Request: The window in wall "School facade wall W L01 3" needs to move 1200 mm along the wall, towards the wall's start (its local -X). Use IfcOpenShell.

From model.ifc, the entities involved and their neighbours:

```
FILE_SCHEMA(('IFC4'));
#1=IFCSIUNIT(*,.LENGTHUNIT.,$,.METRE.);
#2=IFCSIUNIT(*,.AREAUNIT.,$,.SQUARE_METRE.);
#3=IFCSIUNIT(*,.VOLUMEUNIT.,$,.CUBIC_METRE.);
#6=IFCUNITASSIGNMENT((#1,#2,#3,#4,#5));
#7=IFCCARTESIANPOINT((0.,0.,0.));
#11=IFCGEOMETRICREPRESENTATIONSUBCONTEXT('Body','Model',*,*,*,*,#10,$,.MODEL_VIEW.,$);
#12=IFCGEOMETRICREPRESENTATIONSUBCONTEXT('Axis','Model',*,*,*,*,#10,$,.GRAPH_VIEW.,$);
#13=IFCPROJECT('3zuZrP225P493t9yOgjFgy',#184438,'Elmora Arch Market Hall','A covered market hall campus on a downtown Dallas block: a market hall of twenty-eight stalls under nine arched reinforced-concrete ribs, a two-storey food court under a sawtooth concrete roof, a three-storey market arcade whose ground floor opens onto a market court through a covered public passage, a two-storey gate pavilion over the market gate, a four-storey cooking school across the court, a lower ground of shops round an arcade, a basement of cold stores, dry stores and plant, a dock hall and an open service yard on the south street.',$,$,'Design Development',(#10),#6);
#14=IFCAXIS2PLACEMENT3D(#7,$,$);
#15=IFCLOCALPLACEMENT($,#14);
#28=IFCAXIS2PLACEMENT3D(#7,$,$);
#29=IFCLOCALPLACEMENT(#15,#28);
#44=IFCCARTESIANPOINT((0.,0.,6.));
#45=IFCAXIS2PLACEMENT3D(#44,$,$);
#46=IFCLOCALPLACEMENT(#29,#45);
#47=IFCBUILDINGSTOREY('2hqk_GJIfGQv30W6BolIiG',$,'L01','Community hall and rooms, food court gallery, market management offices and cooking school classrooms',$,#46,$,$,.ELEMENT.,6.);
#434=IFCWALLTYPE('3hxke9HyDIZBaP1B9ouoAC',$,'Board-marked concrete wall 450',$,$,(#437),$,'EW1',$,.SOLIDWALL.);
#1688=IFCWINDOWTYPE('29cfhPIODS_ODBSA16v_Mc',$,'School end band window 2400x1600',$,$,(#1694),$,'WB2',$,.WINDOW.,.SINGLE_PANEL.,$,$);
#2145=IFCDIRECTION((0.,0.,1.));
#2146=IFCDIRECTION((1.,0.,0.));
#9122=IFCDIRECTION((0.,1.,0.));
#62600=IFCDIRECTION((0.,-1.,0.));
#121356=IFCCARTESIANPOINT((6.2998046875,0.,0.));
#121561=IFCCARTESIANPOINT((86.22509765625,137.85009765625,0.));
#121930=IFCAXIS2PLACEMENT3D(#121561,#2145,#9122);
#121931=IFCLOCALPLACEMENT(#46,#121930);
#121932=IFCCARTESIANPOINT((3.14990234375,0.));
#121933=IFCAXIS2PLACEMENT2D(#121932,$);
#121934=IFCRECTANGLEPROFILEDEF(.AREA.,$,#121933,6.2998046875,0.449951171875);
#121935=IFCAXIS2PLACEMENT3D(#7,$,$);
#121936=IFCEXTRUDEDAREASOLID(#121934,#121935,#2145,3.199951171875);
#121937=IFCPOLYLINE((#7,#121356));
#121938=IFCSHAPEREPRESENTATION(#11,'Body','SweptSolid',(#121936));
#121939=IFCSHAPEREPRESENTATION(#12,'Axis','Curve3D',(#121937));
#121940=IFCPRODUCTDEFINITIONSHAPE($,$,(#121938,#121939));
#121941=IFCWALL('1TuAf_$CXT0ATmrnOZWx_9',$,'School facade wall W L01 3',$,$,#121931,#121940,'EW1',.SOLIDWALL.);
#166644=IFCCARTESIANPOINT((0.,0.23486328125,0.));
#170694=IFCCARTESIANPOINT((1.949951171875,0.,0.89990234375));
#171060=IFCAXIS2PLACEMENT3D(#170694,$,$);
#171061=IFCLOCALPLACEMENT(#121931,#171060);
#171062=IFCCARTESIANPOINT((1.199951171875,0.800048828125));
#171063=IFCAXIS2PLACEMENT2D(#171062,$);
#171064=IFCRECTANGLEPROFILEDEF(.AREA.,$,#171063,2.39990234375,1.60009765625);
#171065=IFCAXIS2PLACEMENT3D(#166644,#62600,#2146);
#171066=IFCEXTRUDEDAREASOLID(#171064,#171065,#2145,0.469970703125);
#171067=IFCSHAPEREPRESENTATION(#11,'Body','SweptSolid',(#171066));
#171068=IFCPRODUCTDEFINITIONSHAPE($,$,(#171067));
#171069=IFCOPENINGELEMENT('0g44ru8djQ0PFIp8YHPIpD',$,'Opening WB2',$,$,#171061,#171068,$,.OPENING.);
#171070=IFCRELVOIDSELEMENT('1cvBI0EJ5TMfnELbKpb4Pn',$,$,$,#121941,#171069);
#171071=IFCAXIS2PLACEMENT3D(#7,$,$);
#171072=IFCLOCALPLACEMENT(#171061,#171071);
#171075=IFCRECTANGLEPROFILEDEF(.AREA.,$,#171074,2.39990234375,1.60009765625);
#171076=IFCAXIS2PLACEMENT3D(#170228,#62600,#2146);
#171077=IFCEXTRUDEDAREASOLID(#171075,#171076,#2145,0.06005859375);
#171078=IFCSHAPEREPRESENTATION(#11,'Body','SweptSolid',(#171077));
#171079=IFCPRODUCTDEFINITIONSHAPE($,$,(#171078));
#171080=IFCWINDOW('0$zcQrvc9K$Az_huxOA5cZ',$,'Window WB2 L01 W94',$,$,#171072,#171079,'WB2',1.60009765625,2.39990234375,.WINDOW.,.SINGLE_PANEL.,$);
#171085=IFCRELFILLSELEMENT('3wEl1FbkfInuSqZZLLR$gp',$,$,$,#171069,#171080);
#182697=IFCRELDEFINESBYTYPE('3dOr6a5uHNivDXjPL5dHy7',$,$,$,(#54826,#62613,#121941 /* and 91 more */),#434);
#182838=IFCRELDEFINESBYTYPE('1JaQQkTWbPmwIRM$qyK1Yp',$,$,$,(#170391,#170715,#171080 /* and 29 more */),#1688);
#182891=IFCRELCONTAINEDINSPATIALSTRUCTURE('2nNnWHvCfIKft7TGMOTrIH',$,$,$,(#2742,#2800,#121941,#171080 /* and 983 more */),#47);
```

```python
import ifcopenshell
import ifcopenshell.api.geometry
import ifcopenshell.util.placement

model = ifcopenshell.open("model.ifc")

window = model.by_guid("0$zcQrvc9K$Az_huxOA5cZ")
opening = window.FillsVoids[0].RelatingOpeningElement
wall = opening.VoidsElements[0].RelatingBuildingElement

wall_matrix = ifcopenshell.util.placement.get_local_placement(wall.ObjectPlacement)
shift = wall_matrix[:3, 0] * -1.2
before = ifcopenshell.util.placement.get_local_placement(window.ObjectPlacement)[:3, 3].copy()

# The window is placed relative to its opening, so it follows when the opening moves.
matrix = ifcopenshell.util.placement.get_local_placement(opening.ObjectPlacement)
matrix[:3, 3] += shift
ifcopenshell.api.geometry.edit_object_placement(
    model, product=opening, matrix=matrix, is_si=False, should_transform_children=True
)

after = ifcopenshell.util.placement.get_local_placement(window.ObjectPlacement)[:3, 3]
print("window moved by", (after - before).round(3) + 0.0)

model.write("model_edited.ifc")
```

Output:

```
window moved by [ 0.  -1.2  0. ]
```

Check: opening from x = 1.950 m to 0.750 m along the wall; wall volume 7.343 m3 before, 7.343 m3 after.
